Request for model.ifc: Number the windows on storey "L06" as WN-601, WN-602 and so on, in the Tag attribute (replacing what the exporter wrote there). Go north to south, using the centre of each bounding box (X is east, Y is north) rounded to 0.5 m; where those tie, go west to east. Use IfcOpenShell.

First a look at what the model holds.

```python
import ifcopenshell
import ifcopenshell.util.element
import ifcopenshell.util.placement

model = ifcopenshell.open("model.ifc")
print(model.schema)
storey = next(s for s in model.by_type("IfcBuildingStorey") if s.Name == "L06")
windows = [e for e in ifcopenshell.util.element.get_decomposition(storey) if e.is_a("IfcWindow")]
for e in sorted(windows, key=lambda e: e.id()):
    origin = ifcopenshell.util.placement.get_local_placement(e.ObjectPlacement)[:3, 3]
    print(e.id(), e.Tag, e.Name, origin.round(2) + 0.0, sep=" | ")
```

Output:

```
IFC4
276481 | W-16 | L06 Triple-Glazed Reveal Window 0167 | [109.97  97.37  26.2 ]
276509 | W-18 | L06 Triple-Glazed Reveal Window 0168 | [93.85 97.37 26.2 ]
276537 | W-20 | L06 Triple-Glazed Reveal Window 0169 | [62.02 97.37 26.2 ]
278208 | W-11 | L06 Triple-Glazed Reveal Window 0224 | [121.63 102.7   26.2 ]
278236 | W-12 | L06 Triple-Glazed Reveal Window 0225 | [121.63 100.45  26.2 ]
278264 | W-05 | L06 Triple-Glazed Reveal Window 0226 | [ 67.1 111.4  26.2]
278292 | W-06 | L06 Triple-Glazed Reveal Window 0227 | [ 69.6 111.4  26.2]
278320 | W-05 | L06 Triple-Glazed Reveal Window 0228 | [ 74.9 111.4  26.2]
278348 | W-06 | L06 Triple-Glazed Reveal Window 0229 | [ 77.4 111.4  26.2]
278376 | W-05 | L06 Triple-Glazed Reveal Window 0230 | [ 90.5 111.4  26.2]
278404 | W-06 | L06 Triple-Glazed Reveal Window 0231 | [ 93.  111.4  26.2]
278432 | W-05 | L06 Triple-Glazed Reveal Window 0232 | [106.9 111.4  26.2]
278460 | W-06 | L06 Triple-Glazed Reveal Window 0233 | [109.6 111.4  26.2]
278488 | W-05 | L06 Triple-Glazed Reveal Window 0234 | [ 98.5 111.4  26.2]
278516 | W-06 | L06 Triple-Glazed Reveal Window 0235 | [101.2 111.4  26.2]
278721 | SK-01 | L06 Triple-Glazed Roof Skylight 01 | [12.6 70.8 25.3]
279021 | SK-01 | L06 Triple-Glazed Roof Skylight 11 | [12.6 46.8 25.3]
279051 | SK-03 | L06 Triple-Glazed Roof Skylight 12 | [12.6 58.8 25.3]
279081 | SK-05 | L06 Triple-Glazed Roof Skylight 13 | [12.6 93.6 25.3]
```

```python
import ifcopenshell
import ifcopenshell.geom
import ifcopenshell.util.element
import ifcopenshell.util.shape

model = ifcopenshell.open("model.ifc")
settings = ifcopenshell.geom.settings()
settings.set("use-world-coords", True)


def centre(element):
    shape = ifcopenshell.geom.create_shape(settings, element)
    return ifcopenshell.util.shape.get_bbox_centroid(shape.geometry)


storey = next(s for s in model.by_type("IfcBuildingStorey") if s.Name == "L06")
windows = [e for e in ifcopenshell.util.element.get_decomposition(storey) if e.is_a("IfcWindow")]

# Insertion points can sit at a corner or the storey origin, so sort by the geometry (in metres).
centres = {e: centre(e) for e in windows}
windows.sort(key=lambda e: (-round(centres[e][1] / 0.5), centres[e][0]))

for i, e in enumerate(windows, start=1):
    number = f"WN-6{i:02d}"
    e.Tag = number
    print(e.id(), number)

model.write("model_rev.ifc")
```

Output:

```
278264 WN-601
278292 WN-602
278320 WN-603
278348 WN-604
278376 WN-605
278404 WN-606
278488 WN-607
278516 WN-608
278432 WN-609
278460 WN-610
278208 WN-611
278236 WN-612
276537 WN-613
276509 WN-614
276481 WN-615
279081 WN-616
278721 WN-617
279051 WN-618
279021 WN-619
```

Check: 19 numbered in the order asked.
